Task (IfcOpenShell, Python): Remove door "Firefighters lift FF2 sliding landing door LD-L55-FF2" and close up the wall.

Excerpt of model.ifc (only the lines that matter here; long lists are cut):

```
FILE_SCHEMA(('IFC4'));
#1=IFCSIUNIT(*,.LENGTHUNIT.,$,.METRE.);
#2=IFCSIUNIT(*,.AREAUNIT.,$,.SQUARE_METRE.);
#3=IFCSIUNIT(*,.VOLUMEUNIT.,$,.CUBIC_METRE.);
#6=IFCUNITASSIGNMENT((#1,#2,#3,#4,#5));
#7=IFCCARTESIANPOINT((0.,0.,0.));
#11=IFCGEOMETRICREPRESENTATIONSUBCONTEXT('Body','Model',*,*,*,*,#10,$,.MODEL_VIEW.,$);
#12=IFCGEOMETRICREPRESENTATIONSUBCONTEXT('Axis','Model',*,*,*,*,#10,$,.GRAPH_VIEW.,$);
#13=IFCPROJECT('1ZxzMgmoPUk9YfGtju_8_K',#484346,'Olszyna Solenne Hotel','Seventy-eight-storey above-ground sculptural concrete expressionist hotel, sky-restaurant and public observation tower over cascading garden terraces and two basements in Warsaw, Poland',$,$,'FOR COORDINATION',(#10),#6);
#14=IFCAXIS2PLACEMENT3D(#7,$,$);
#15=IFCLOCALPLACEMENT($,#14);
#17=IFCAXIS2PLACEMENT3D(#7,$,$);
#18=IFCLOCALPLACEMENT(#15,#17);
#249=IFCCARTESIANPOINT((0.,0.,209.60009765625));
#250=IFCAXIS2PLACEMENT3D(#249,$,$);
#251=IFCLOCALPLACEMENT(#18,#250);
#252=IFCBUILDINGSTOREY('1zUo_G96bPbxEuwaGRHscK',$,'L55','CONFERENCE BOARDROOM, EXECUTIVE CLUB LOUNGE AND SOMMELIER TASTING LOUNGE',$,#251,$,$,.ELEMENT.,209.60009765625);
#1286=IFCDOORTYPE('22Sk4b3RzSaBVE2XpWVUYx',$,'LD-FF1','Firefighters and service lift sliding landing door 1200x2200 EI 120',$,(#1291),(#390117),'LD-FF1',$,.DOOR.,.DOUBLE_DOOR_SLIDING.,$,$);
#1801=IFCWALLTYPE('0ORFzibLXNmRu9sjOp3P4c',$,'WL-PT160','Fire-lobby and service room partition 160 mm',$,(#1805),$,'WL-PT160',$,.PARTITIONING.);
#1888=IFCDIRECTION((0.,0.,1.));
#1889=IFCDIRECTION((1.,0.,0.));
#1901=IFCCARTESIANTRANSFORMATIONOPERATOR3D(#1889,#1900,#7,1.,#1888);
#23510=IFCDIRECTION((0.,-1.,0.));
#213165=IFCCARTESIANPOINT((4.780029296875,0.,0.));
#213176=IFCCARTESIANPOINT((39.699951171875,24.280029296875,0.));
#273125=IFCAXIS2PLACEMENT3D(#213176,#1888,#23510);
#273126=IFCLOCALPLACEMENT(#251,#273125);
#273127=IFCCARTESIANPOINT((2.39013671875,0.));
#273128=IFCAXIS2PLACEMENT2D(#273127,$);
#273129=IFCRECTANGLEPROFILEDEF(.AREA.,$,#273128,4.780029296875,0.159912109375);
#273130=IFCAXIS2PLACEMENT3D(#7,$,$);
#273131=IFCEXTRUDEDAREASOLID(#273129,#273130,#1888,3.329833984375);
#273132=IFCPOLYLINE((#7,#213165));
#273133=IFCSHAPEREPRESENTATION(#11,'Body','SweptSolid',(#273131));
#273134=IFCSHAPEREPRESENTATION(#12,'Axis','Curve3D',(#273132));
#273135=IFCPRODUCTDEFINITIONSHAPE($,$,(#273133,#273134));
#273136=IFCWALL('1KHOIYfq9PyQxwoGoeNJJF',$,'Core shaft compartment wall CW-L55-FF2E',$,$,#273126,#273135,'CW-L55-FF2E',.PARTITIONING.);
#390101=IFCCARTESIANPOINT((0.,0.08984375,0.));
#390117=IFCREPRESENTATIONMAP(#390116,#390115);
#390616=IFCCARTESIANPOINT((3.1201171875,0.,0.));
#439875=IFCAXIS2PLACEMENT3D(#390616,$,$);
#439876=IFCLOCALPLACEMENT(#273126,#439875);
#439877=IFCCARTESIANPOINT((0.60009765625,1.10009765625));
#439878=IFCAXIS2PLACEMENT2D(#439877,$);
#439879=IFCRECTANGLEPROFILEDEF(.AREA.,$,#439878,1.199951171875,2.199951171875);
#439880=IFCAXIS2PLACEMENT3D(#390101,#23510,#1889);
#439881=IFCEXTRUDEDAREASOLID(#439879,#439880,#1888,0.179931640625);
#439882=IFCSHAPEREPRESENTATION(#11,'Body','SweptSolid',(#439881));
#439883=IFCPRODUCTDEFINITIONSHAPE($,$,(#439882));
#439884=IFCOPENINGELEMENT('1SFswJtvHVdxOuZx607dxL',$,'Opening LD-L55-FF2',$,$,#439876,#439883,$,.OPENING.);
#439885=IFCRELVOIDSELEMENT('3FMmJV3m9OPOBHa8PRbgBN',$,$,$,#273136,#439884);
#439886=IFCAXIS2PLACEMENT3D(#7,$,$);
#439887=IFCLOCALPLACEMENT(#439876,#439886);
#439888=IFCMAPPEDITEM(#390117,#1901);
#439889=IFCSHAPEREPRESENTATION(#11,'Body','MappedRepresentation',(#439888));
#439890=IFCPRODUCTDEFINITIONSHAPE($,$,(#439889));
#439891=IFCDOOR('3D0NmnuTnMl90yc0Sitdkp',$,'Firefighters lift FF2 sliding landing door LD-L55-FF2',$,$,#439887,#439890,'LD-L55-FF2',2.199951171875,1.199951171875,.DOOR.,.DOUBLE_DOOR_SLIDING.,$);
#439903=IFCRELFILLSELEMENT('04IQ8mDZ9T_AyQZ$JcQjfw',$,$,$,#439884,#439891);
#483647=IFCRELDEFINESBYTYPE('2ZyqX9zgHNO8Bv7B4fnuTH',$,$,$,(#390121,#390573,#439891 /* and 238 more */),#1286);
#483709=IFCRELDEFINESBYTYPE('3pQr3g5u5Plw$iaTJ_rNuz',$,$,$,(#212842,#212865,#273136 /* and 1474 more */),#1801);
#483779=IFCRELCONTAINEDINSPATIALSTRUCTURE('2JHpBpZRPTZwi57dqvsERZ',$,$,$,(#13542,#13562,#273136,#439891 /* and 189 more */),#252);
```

```python
import ifcopenshell
import ifcopenshell.api.feature
import ifcopenshell.api.root
import ifcopenshell.geom
import ifcopenshell.util.shape

model = ifcopenshell.open("model.ifc")
settings = ifcopenshell.geom.settings()


def volume(element):
    """Net volume in cubic metres, openings subtracted."""
    shape = ifcopenshell.geom.create_shape(settings, element)
    return ifcopenshell.util.shape.get_volume(shape.geometry)


door = model.by_guid("3D0NmnuTnMl90yc0Sitdkp")
opening = door.FillsVoids[0].RelatingOpeningElement
wall = opening.VoidsElements[0].RelatingBuildingElement
before = volume(wall)

ifcopenshell.api.root.remove_product(model, product=door)
ifcopenshell.api.feature.remove_feature(model, feature=opening)

after = volume(wall)

print(f"wall volume {before:.3f} -> {after:.3f} m3")

model.write("model_v2.ifc")
```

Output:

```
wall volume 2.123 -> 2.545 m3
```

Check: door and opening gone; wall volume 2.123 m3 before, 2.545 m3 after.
